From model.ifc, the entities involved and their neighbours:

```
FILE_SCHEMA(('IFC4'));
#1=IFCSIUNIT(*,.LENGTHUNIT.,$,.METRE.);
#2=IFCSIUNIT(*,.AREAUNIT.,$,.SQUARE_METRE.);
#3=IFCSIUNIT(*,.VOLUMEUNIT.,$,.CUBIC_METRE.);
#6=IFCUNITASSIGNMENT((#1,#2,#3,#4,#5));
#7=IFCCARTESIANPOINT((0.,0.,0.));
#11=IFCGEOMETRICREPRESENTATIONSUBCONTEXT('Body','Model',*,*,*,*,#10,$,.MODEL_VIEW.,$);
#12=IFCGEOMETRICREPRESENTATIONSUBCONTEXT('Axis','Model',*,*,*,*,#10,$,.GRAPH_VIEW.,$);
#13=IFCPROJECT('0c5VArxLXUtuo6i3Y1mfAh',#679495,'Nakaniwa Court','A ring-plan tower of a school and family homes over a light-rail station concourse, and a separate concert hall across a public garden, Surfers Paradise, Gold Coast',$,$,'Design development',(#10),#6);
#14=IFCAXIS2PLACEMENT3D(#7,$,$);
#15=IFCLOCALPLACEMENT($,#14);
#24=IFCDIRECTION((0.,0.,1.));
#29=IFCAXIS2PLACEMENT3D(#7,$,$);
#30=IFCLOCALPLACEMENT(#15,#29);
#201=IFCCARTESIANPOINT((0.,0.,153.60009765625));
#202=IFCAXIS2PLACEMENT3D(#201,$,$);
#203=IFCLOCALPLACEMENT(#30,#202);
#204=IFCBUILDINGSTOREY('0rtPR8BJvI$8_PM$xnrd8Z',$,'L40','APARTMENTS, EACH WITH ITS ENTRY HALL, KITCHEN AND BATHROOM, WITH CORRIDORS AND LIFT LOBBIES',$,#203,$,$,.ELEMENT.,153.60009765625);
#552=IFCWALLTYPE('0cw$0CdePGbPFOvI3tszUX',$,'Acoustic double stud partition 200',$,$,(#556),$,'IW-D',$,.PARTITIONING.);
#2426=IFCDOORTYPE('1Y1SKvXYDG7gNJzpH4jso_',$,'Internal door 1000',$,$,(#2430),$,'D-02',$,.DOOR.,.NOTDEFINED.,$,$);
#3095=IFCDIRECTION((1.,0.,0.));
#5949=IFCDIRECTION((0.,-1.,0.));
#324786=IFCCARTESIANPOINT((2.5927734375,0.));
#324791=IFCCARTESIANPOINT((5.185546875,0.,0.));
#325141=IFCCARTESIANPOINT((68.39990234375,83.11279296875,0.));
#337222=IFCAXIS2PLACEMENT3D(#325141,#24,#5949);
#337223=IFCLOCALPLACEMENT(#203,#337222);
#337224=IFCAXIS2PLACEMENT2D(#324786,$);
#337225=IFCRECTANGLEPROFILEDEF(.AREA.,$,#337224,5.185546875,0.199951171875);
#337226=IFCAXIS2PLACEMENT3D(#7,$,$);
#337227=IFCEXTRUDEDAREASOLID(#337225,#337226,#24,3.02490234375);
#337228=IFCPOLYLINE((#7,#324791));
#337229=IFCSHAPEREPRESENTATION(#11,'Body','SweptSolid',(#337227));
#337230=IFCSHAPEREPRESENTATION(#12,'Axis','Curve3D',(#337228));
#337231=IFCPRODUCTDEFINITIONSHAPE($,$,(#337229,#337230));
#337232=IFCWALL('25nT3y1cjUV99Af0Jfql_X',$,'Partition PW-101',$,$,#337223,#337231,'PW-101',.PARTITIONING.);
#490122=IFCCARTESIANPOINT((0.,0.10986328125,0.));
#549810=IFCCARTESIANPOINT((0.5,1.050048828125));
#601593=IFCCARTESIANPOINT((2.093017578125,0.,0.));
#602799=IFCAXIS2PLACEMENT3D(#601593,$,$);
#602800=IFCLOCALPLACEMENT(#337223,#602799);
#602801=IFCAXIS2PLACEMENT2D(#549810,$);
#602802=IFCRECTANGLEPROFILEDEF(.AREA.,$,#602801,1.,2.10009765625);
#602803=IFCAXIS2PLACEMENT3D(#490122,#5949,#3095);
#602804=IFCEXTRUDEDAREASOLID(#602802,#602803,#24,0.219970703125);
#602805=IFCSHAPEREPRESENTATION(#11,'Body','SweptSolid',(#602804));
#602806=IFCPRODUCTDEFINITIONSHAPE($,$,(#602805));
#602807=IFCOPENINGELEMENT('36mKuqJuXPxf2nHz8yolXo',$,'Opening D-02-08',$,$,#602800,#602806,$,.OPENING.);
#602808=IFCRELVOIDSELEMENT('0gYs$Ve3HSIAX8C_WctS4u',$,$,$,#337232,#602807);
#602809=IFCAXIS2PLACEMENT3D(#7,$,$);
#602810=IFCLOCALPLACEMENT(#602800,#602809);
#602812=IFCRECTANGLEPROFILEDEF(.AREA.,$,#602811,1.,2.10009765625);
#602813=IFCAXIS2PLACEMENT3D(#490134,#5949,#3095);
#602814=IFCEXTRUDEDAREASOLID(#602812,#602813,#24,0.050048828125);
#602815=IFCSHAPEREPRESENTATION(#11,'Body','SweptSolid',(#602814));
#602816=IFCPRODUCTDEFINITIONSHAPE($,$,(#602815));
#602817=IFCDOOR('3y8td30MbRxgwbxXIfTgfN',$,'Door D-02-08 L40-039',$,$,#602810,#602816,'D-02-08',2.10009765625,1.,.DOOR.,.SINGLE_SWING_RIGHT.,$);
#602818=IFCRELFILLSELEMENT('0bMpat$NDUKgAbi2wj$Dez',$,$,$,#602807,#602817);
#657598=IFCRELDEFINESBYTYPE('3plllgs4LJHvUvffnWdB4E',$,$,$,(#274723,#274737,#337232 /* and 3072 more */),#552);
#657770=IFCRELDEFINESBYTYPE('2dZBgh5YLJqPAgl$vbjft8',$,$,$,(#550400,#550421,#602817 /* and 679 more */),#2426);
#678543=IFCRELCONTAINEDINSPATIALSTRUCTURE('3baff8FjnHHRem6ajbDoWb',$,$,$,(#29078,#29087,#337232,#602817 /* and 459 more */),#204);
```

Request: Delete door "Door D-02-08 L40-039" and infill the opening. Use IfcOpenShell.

```python
import ifcopenshell
import ifcopenshell.api.feature
import ifcopenshell.api.root
import ifcopenshell.geom
import ifcopenshell.util.shape

model = ifcopenshell.open("model.ifc")
settings = ifcopenshell.geom.settings()


def volume(element):
    """Net volume in cubic metres, openings subtracted."""
    shape = ifcopenshell.geom.create_shape(settings, element)
    return ifcopenshell.util.shape.get_volume(shape.geometry)


door = model.by_guid("3y8td30MbRxgwbxXIfTgfN")
opening = door.FillsVoids[0].RelatingOpeningElement
wall = opening.VoidsElements[0].RelatingBuildingElement
before = volume(wall)

ifcopenshell.api.root.remove_product(model, product=door)
ifcopenshell.api.feature.remove_feature(model, feature=opening)

after = volume(wall)

print(f"wall volume {before:.3f} -> {after:.3f} m3")

model.write("model_updated.ifc")
```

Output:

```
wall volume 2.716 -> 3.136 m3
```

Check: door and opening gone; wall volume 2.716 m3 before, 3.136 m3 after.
